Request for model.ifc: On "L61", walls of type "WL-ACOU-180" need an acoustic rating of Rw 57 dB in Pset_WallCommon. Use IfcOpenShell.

First a look at what the model holds.

```python
import ifcopenshell
import ifcopenshell.util.element

model = ifcopenshell.open("model.ifc")
print(model.schema)
storey = next(s for s in model.by_type("IfcBuildingStorey") if s.Name == "L61")
walls = [e for e in ifcopenshell.util.element.get_decomposition(storey) if e.is_a("IfcWall")]
seen = {}
for e in walls:
    element_type = ifcopenshell.util.element.get_type(e)
    key = (element_type.Name if element_type != e and element_type else None, ifcopenshell.util.element.get_pset(e, "Pset_WallCommon", "AcousticRating"))
    seen[key] = seen.get(key, 0) + 1
for (name, value), count in sorted(seen.items(), key=str):
    print(count, "x", name, "|", value)
```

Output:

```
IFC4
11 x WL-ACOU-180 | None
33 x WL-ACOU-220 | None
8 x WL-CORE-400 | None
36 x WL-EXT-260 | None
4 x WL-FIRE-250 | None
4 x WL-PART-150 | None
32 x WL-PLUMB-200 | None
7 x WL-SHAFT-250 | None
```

```python
import ifcopenshell
import ifcopenshell.api.pset
import ifcopenshell.util.element

model = ifcopenshell.open("model.ifc")

storey = next(s for s in model.by_type("IfcBuildingStorey") if s.Name == "L61")
walls = [e for e in ifcopenshell.util.element.get_decomposition(storey) if e.is_a("IfcWall")]

count = 0
for e in walls:
    element_type = ifcopenshell.util.element.get_type(e)
    if element_type in (None, e) or element_type.Name != "WL-ACOU-180":
        continue
    found = ifcopenshell.util.element.get_pset(e, "Pset_WallCommon", should_inherit=False)
    if found:
        pset = model.by_id(found["id"])
        if len(ifcopenshell.util.element.get_elements_by_pset(pset)) > 1:
            pset = ifcopenshell.api.pset.unshare_pset(model, products=[e], pset=pset)[0]
    else:
        pset = ifcopenshell.api.pset.add_pset(model, product=e, name="Pset_WallCommon")
    ifcopenshell.api.pset.edit_pset(model, pset=pset, properties={"AcousticRating": "Rw 57 dB"})
    count += 1

print(count, "walls updated")

model.write("model_edited.ifc")
```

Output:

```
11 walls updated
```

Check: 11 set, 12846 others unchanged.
